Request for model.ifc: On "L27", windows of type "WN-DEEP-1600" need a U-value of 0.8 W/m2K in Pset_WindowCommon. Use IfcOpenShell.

First a look at what the model holds.

```python
import ifcopenshell
import ifcopenshell.util.element

model = ifcopenshell.open("model.ifc")
print(model.schema)
storey = next(s for s in model.by_type("IfcBuildingStorey") if s.Name == "L27")
windows = [e for e in ifcopenshell.util.element.get_decomposition(storey) if e.is_a("IfcWindow")]
seen = {}
for e in windows:
    element_type = ifcopenshell.util.element.get_type(e)
    key = (element_type.Name if element_type != e and element_type else None, ifcopenshell.util.element.get_pset(e, "Pset_WindowCommon", "ThermalTransmittance"))
    seen[key] = seen.get(key, 0) + 1
for (name, value), count in sorted(seen.items(), key=str):
    print(count, "x", name, "|", value)
```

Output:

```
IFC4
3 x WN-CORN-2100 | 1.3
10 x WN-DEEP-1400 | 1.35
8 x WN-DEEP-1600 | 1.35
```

```python
import ifcopenshell
import ifcopenshell.api.pset
import ifcopenshell.util.element

model = ifcopenshell.open("model.ifc")

storey = next(s for s in model.by_type("IfcBuildingStorey") if s.Name == "L27")
windows = [e for e in ifcopenshell.util.element.get_decomposition(storey) if e.is_a("IfcWindow")]

count = 0
for e in windows:
    element_type = ifcopenshell.util.element.get_type(e)
    if element_type in (None, e) or element_type.Name != "WN-DEEP-1600":
        continue
    found = ifcopenshell.util.element.get_pset(e, "Pset_WindowCommon", should_inherit=False)
    if found:
        pset = model.by_id(found["id"])
        if len(ifcopenshell.util.element.get_elements_by_pset(pset)) > 1:
            pset = ifcopenshell.api.pset.unshare_pset(model, products=[e], pset=pset)[0]
    else:
        pset = ifcopenshell.api.pset.add_pset(model, product=e, name="Pset_WindowCommon")
    ifcopenshell.api.pset.edit_pset(model, pset=pset, properties={"ThermalTransmittance": 0.8})
    count += 1

print(count, "windows updated")

model.write("model_updated.ifc")
```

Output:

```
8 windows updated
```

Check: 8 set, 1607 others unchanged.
